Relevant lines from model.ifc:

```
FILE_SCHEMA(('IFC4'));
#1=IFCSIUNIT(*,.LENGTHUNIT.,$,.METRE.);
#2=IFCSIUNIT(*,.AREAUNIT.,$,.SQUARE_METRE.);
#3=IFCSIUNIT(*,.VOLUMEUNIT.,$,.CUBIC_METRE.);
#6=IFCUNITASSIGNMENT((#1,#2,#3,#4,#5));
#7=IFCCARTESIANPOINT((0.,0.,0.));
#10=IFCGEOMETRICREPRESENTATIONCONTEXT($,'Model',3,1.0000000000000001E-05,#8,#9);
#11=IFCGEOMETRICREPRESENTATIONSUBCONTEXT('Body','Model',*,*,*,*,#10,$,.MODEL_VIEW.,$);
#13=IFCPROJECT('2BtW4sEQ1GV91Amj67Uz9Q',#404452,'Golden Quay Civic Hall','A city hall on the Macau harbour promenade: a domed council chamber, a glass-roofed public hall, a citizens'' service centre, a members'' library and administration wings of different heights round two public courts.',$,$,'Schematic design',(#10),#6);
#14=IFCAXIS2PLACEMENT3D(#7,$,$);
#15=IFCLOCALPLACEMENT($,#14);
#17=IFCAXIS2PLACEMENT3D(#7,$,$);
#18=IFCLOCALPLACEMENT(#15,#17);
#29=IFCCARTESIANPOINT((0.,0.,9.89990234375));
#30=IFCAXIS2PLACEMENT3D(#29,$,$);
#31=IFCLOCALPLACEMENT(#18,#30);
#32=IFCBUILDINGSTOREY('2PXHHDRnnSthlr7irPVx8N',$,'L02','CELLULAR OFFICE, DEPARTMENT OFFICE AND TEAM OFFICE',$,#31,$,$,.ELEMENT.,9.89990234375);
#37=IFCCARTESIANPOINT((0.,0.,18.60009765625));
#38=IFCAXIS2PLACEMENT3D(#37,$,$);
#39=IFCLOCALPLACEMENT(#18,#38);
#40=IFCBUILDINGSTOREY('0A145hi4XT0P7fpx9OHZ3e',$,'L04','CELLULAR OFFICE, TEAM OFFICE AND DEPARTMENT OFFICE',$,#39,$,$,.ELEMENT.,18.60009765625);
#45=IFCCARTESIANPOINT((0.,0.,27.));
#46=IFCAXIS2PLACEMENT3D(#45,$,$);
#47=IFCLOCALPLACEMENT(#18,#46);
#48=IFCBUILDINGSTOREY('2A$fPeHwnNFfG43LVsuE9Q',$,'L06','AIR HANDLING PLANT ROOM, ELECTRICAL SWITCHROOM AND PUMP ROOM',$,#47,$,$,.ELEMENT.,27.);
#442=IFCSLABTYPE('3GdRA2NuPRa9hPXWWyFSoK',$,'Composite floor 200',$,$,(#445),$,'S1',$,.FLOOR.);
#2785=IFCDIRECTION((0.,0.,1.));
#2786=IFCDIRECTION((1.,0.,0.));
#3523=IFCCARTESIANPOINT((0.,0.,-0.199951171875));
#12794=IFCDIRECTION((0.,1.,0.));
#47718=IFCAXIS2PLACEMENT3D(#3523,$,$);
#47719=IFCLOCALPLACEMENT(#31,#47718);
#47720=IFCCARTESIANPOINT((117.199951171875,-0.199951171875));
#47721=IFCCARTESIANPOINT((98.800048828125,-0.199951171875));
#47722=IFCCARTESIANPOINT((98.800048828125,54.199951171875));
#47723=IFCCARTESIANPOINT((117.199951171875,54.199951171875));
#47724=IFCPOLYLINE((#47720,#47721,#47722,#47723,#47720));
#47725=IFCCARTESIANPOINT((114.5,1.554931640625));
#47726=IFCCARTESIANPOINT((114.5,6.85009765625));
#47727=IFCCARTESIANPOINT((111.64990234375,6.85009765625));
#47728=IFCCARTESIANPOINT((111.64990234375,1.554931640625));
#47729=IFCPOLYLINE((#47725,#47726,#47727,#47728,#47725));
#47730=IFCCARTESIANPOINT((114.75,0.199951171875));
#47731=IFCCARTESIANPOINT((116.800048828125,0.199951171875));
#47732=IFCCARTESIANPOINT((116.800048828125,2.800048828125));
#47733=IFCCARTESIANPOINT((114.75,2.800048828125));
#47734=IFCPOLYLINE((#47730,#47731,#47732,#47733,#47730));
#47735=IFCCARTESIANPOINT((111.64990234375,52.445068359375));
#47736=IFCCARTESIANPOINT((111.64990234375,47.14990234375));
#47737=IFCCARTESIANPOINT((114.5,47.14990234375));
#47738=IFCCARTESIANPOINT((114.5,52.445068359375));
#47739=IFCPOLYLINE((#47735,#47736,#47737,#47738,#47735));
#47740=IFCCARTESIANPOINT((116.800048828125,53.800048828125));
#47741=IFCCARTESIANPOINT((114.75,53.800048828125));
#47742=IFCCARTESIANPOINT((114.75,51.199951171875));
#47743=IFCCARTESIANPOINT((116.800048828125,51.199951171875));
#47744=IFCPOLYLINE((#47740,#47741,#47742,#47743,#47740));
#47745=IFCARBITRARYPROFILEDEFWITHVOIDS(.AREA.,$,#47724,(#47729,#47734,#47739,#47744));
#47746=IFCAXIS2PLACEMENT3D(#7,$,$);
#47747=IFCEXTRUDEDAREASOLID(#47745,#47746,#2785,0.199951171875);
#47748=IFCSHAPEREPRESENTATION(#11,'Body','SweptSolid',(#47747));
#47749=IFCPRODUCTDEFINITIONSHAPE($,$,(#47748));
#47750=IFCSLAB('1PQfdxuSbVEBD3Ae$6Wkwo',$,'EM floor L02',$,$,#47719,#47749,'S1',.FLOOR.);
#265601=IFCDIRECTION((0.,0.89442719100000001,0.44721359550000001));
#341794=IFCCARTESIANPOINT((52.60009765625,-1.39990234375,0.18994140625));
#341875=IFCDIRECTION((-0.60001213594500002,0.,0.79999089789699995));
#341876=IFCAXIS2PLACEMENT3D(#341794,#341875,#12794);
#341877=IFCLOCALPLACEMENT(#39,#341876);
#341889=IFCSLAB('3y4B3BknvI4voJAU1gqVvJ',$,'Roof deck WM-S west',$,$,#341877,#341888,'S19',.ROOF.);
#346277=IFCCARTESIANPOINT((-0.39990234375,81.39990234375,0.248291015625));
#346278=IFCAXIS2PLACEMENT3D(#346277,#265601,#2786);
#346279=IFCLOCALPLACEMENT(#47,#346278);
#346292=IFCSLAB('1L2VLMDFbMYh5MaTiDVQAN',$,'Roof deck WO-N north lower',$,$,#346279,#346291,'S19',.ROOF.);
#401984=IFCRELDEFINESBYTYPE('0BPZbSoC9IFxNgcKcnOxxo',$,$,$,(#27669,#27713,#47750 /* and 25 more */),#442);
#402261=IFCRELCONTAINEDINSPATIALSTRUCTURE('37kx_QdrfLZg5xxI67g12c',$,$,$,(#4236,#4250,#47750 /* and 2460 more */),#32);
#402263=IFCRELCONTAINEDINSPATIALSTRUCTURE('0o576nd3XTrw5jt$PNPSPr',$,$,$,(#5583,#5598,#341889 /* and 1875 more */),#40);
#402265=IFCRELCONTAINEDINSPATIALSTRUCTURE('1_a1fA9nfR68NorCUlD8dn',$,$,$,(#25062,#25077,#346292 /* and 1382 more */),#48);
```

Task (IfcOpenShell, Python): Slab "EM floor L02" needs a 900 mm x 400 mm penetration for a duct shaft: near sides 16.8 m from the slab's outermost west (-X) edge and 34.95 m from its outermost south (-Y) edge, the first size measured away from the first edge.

```python
import numpy as np
import ifcopenshell
import ifcopenshell.api.feature
import ifcopenshell.api.geometry
import ifcopenshell.api.root
import ifcopenshell.geom
import ifcopenshell.util.placement
import ifcopenshell.util.representation
import ifcopenshell.util.shape
import ifcopenshell.util.unit

model = ifcopenshell.open("model.ifc")
unit_scale = ifcopenshell.util.unit.calculate_unit_scale(model)
settings = ifcopenshell.geom.settings()


def volume(element):
    """Net volume in cubic metres, openings subtracted."""
    shape = ifcopenshell.geom.create_shape(settings, element)
    return ifcopenshell.util.shape.get_volume(shape.geometry)


slab = model.by_guid("1PQfdxuSbVEBD3Ae$6Wkwo")
before = volume(slab)

# Extent in the slab's own axes, in metres. The edges named are its -X and -Y sides.
slab_shape = ifcopenshell.geom.create_shape(settings, slab)
vertices = ifcopenshell.util.shape.get_vertices(slab_shape.geometry)
x_min, y_min, bottom = vertices.min(axis=0)
top = vertices[:, 2].max()

opening = ifcopenshell.api.root.create_entity(model, ifc_class="IfcOpeningElement", name="Duct shaft opening", predefined_type="OPENING")
context = ifcopenshell.util.representation.get_context(model, "Model", "Body", "MODEL_VIEW")
width, depth = 0.9, 0.4
outline = [(0.0, 0.0), (width, 0.0), (width, depth), (0.0, depth), (0.0, 0.0)]
# Overshoot both faces by 50 mm so the cut is clean.
shape = ifcopenshell.api.geometry.add_slab_representation(
    model, context=context, depth=top - bottom + 0.1, polyline=outline
)
ifcopenshell.api.geometry.assign_representation(model, product=opening, representation=shape)

matrix = ifcopenshell.util.placement.get_local_placement(slab.ObjectPlacement)
matrix[:, 3] = matrix @ np.append(np.array([x_min + 16.8, y_min + 34.95, bottom - 0.05]) / unit_scale, 1.0)
ifcopenshell.api.geometry.edit_object_placement(model, product=opening, matrix=matrix, is_si=False)
ifcopenshell.api.feature.add_feature(model, feature=opening, element=slab)

after = volume(slab)

print(f"slab volume {before:.3f} -> {after:.3f} m3")

model.write("model_updated.ifc")
```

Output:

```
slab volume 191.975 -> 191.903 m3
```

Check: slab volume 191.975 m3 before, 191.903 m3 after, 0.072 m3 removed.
